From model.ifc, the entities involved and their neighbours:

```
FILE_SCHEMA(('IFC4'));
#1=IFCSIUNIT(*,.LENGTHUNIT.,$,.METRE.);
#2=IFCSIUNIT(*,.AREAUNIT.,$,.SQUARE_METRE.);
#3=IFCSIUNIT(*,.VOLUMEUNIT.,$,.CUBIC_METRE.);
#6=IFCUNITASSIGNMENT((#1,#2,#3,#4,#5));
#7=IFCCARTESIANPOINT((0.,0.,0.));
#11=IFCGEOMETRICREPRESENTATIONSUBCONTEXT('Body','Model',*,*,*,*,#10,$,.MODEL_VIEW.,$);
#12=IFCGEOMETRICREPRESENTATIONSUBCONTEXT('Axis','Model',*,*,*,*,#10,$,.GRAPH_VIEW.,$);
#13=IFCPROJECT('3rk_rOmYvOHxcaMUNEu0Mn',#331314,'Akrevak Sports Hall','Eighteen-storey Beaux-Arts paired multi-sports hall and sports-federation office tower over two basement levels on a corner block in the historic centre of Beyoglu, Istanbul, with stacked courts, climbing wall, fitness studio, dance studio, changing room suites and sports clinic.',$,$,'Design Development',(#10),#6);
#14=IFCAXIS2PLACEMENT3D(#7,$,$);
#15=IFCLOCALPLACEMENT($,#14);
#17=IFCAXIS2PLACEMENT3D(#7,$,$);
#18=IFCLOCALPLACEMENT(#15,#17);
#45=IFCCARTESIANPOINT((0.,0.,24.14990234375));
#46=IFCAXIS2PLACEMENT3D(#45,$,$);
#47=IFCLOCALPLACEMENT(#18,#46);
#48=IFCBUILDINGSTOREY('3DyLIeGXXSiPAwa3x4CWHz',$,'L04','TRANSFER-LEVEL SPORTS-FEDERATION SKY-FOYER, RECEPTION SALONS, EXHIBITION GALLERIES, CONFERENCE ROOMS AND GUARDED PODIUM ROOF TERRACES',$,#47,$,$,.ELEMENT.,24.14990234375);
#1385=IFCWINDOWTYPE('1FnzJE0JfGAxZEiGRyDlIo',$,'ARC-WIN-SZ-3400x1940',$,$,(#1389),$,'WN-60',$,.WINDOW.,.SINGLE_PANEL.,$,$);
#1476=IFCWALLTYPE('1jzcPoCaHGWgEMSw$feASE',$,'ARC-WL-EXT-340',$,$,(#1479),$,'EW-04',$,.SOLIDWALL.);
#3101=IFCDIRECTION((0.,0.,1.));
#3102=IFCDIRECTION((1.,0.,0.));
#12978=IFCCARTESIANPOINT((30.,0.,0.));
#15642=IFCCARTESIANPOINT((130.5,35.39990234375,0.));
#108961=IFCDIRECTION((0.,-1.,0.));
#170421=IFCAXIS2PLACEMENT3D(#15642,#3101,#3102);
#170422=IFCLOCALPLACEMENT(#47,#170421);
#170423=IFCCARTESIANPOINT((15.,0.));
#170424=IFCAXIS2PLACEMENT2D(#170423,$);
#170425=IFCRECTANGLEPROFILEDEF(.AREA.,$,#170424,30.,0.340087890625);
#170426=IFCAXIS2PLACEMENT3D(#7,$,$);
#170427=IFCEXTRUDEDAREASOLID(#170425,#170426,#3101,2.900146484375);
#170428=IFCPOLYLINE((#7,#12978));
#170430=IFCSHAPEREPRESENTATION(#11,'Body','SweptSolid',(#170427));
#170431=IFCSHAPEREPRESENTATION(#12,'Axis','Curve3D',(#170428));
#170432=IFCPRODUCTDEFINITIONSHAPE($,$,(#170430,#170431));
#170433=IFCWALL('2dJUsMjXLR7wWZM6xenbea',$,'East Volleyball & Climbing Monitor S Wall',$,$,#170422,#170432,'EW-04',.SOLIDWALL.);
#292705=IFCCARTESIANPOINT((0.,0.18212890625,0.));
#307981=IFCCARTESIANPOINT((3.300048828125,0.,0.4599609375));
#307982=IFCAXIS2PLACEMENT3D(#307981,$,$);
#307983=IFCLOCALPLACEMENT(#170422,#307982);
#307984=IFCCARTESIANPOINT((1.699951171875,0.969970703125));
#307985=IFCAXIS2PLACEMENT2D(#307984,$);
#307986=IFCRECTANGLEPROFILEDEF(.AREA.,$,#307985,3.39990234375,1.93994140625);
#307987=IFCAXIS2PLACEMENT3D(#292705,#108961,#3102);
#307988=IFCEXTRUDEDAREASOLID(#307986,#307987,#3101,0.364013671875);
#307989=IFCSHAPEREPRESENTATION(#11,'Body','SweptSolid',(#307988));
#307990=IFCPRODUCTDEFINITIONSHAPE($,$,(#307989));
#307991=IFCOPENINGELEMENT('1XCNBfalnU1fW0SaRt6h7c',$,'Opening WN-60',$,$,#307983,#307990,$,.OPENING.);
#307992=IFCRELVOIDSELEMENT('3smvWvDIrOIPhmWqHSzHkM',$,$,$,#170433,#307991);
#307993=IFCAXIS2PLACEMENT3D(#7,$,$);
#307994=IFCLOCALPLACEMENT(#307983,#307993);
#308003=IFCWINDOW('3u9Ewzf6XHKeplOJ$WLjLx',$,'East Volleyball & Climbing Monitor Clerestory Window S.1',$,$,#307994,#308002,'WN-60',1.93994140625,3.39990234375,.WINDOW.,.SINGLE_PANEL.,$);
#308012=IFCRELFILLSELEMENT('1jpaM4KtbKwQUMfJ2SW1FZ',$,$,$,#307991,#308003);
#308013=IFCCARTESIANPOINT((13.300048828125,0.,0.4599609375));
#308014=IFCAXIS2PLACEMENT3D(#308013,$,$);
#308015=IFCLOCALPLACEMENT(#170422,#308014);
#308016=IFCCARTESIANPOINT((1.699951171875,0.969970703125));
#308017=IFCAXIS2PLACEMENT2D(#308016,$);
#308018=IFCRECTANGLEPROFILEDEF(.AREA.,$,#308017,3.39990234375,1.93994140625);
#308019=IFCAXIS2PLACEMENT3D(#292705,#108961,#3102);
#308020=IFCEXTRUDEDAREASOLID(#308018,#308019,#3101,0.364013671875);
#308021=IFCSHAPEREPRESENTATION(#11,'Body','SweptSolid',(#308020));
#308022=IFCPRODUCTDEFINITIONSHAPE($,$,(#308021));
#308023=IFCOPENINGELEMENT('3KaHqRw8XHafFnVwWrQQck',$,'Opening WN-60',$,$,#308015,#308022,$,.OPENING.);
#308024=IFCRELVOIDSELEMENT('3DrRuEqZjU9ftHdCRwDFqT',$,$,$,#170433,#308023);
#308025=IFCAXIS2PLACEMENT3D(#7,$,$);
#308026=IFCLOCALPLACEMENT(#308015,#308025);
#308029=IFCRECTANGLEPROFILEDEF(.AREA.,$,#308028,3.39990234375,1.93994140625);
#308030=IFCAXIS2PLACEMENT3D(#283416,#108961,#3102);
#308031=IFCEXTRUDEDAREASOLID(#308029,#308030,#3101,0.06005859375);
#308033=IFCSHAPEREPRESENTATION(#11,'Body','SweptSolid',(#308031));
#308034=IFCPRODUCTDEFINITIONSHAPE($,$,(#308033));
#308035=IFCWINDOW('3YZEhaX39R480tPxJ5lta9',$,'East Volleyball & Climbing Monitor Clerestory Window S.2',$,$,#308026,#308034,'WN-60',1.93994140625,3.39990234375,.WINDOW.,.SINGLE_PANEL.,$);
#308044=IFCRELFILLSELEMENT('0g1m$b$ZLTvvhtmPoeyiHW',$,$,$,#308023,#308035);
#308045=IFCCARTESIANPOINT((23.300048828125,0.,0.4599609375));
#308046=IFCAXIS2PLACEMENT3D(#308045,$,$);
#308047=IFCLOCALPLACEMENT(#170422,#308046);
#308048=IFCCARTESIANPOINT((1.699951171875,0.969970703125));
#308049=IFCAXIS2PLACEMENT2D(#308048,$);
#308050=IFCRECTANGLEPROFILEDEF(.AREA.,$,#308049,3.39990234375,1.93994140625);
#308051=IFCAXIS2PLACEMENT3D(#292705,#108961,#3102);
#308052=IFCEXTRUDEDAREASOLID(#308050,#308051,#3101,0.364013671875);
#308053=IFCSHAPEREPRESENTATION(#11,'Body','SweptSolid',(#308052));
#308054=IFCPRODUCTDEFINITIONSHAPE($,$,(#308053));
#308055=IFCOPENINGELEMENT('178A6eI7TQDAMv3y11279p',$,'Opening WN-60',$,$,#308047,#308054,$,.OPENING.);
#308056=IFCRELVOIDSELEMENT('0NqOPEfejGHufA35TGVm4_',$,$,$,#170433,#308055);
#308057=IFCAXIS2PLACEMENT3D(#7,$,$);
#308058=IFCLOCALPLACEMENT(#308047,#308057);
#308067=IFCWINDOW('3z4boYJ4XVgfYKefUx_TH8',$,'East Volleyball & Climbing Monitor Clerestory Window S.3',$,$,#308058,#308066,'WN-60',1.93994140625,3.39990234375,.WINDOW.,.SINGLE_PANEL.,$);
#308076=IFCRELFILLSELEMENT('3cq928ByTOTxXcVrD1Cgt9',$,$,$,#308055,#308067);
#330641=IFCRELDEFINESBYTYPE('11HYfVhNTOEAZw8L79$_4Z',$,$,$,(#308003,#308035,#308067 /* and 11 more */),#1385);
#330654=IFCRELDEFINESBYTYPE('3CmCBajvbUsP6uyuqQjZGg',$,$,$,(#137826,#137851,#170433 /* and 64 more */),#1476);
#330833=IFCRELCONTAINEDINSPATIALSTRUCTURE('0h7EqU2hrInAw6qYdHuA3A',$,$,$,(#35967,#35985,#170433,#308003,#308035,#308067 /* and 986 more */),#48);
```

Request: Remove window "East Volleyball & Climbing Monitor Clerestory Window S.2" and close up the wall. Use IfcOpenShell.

```python
import ifcopenshell
import ifcopenshell.api.feature
import ifcopenshell.api.root
import ifcopenshell.geom
import ifcopenshell.util.shape

model = ifcopenshell.open("model.ifc")
settings = ifcopenshell.geom.settings()


def volume(element):
    """Net volume in cubic metres, openings subtracted."""
    shape = ifcopenshell.geom.create_shape(settings, element)
    return ifcopenshell.util.shape.get_volume(shape.geometry)


window = model.by_id(308035)
opening = window.FillsVoids[0].RelatingOpeningElement
wall = opening.VoidsElements[0].RelatingBuildingElement
before = volume(wall)

ifcopenshell.api.root.remove_product(model, product=window)
ifcopenshell.api.feature.remove_feature(model, feature=opening)

after = volume(wall)

print(f"wall volume {before:.3f} -> {after:.3f} m3")

model.write("model_rev.ifc")
```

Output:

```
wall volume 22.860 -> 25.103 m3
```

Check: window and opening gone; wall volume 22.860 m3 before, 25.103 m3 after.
